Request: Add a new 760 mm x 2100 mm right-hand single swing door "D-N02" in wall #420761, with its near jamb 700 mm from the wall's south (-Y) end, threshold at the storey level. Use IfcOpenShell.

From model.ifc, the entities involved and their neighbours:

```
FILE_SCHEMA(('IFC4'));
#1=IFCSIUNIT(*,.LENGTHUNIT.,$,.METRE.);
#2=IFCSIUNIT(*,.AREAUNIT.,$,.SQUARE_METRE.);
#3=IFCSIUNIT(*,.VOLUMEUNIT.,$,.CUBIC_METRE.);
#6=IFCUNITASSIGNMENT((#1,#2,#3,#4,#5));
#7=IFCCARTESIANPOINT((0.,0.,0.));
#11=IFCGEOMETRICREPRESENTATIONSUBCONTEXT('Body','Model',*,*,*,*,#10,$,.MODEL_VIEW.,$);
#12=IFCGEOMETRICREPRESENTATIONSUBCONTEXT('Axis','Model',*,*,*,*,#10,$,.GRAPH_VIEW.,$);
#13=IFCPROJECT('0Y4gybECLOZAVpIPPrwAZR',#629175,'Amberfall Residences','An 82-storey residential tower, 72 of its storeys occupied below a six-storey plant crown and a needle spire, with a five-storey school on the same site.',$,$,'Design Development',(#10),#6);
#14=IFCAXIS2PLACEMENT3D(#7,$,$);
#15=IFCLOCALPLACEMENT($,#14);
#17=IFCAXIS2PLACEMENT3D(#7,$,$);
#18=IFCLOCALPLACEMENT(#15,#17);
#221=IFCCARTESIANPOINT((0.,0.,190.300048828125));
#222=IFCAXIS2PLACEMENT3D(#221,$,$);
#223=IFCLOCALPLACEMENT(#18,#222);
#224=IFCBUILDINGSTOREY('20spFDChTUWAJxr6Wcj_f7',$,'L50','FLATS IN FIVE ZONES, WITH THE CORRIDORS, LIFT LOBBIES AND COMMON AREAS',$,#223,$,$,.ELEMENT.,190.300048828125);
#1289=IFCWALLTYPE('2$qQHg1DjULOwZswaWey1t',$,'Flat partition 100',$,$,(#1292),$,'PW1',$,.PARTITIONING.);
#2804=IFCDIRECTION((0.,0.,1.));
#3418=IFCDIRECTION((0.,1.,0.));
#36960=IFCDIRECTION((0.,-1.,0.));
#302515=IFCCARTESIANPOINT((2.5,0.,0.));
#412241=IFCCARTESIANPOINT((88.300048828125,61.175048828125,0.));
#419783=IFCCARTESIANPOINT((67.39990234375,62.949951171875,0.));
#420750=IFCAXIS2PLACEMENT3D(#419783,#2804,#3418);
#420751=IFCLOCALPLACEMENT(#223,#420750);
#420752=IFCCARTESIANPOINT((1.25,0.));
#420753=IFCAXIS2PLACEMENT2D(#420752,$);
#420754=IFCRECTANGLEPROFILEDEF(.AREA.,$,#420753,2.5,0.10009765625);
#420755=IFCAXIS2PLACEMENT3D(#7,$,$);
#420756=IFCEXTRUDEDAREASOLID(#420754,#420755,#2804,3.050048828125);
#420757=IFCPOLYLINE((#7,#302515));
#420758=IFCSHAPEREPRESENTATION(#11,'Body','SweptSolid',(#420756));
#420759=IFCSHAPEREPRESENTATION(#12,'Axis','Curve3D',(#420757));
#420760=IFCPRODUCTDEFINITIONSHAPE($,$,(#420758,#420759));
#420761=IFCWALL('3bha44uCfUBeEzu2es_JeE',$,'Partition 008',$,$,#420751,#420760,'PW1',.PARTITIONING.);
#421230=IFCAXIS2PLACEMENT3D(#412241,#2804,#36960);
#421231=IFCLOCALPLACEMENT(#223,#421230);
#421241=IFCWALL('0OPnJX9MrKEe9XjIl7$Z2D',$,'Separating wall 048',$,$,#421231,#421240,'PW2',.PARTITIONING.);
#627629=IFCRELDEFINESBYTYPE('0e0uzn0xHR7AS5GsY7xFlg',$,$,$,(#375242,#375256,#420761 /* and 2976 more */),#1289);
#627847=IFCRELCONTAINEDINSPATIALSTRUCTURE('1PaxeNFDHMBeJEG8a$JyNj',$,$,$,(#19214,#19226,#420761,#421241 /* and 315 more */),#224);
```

```python
import numpy as np
import ifcopenshell
import ifcopenshell.api.feature
import ifcopenshell.api.geometry
import ifcopenshell.api.root
import ifcopenshell.api.spatial
import ifcopenshell.geom
import ifcopenshell.util.element
import ifcopenshell.util.placement
import ifcopenshell.util.representation
import ifcopenshell.util.shape
import ifcopenshell.util.unit

model = ifcopenshell.open("model.ifc")
unit_scale = ifcopenshell.util.unit.calculate_unit_scale(model)
settings = ifcopenshell.geom.settings()


def volume(element):
    """Net volume in cubic metres, openings subtracted."""
    shape = ifcopenshell.geom.create_shape(settings, element)
    return ifcopenshell.util.shape.get_volume(shape.geometry)


wall = model.by_id(420761)
storey = ifcopenshell.util.element.get_container(wall, ifc_class="IfcBuildingStorey")
context = ifcopenshell.util.representation.get_context(model, "Model", "Body", "MODEL_VIEW")
before = volume(wall)

width, height, from_end, sill = 0.76, 2.1, 0.7, 0.0  # metres

# The wall runs along its own X axis, and the end named is its -X end.
wall_shape = ifcopenshell.geom.create_shape(settings, wall)
x, y, z = ifcopenshell.util.shape.get_vertices(wall_shape.geometry).T
start = x.min() + from_end
face, thickness = float(y.min()), float(y.max() - y.min())
wall_matrix = ifcopenshell.util.placement.get_local_placement(wall.ObjectPlacement)
level = ifcopenshell.util.placement.get_local_placement(storey.ObjectPlacement)[2, 3]


def in_wall(x, y):
    """Placement at x, y metres in the wall's axes, at sill height."""
    matrix = wall_matrix.copy()
    matrix[:, 3] = wall_matrix @ np.array([x / unit_scale, y / unit_scale, 0.0, 1.0])
    matrix[2, 3] = level + sill / unit_scale
    return matrix


# Opening: a box that overshoots both wall faces by 50 mm.
opening = ifcopenshell.api.root.create_entity(model, ifc_class="IfcOpeningElement", predefined_type="OPENING")
box = ifcopenshell.api.geometry.add_wall_representation(
    model, context=context, length=width, height=height, thickness=thickness + 0.1
)
ifcopenshell.api.geometry.assign_representation(model, product=opening, representation=box)
ifcopenshell.api.geometry.edit_object_placement(model, product=opening, matrix=in_wall(start, face - 0.05), is_si=False)
ifcopenshell.api.feature.add_feature(model, feature=opening, element=wall)

door = ifcopenshell.api.root.create_entity(model, ifc_class="IfcDoor", name="D-N02", predefined_type="DOOR")
door.OverallWidth, door.OverallHeight = width / unit_scale, height / unit_scale
door.OperationType = "SINGLE_SWING_RIGHT"
body = ifcopenshell.api.geometry.add_door_representation(
    model,
    context=context,
    overall_width=door.OverallWidth,
    overall_height=door.OverallHeight,
    operation_type="SINGLE_SWING_RIGHT",
    lining_properties={"LiningDepth": thickness / unit_scale, "ThresholdDepth": thickness / unit_scale},
)
ifcopenshell.api.geometry.assign_representation(model, product=door, representation=body)
ifcopenshell.api.spatial.assign_container(model, products=[door], relating_structure=storey)
ifcopenshell.api.feature.add_filling(model, opening=opening, element=door)

# The lining spans the wall, so the door starts at the wall face.
ifcopenshell.api.geometry.edit_object_placement(model, product=door, matrix=in_wall(start, face), is_si=False)

after = volume(wall)

print(f"wall volume {before:.3f} -> {after:.3f} m3")

model.write("model-out.ifc")
```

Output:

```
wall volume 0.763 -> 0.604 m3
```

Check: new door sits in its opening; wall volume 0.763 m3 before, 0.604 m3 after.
